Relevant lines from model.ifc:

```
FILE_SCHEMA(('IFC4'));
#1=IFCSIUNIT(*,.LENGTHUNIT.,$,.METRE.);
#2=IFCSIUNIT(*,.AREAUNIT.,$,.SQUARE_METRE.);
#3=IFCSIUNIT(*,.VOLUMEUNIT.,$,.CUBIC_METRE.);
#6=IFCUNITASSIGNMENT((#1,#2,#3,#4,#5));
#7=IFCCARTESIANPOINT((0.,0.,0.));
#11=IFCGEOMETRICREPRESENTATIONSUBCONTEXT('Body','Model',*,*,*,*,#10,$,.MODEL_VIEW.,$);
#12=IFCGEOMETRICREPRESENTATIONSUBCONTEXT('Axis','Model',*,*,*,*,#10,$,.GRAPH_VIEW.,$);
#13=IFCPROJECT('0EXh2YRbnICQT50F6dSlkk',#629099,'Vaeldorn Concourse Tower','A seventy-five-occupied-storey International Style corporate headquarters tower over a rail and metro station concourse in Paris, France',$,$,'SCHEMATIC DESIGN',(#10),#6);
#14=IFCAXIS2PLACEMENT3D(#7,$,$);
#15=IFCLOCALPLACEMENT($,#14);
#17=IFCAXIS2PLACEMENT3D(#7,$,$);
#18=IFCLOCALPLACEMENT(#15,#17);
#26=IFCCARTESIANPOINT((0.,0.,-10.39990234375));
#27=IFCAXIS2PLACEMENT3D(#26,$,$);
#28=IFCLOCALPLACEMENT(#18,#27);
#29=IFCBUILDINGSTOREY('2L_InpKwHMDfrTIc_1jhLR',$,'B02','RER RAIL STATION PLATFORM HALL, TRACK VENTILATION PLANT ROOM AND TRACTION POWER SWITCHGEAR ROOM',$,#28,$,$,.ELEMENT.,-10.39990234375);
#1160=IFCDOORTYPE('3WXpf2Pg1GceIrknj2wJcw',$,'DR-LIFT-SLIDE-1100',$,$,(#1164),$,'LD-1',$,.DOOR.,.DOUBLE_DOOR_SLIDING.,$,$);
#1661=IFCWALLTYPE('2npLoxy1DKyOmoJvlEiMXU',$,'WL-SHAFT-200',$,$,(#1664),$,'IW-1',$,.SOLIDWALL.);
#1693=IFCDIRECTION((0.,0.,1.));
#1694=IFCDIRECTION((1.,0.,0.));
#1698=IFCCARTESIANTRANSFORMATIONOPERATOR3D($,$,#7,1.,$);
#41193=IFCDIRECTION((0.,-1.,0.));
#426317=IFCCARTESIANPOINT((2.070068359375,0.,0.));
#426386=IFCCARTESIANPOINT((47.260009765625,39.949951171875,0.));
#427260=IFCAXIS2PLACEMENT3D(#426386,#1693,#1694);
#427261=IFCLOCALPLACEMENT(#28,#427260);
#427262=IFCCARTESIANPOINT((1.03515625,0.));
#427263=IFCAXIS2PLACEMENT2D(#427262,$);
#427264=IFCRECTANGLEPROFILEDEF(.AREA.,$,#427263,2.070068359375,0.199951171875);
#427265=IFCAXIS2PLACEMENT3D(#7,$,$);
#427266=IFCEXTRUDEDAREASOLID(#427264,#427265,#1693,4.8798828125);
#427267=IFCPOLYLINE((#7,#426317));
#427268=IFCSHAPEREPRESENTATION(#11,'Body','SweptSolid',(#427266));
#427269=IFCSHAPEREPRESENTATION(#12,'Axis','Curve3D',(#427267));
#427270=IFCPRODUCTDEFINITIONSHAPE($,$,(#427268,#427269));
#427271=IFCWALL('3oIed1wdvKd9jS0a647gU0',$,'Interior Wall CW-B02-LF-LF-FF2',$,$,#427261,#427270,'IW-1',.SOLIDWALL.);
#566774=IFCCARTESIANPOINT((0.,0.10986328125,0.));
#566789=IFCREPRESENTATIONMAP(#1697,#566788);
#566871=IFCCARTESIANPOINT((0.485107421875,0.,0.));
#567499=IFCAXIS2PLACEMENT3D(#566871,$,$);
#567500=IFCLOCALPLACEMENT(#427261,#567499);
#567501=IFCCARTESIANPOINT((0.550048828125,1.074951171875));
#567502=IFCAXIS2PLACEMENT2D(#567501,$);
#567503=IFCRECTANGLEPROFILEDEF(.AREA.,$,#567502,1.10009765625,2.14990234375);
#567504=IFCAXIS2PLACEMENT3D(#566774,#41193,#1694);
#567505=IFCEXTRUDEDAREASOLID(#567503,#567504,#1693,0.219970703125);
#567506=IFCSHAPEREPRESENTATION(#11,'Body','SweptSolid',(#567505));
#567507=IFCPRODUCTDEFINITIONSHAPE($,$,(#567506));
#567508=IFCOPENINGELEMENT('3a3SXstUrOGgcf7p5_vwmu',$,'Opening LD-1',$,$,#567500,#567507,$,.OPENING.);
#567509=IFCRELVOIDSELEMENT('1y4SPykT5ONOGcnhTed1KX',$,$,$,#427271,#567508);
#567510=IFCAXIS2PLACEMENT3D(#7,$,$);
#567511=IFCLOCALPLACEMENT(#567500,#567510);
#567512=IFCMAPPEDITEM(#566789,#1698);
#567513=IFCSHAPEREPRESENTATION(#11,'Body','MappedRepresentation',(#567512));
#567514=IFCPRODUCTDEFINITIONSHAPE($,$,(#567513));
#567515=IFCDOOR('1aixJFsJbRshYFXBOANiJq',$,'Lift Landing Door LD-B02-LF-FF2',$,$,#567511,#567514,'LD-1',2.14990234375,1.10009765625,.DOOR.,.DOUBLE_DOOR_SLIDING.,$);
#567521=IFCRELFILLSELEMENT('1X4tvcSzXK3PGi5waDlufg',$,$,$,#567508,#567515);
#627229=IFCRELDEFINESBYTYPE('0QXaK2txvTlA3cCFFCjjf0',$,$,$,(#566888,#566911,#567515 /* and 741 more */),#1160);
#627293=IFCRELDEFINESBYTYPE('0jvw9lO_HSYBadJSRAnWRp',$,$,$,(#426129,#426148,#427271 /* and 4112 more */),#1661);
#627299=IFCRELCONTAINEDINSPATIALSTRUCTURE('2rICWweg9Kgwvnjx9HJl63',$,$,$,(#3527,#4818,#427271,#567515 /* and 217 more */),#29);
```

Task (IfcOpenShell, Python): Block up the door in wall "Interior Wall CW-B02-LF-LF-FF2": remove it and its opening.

```python
import ifcopenshell
import ifcopenshell.api.feature
import ifcopenshell.api.root
import ifcopenshell.geom
import ifcopenshell.util.shape

model = ifcopenshell.open("model.ifc")
settings = ifcopenshell.geom.settings()


def volume(element):
    """Net volume in cubic metres, openings subtracted."""
    shape = ifcopenshell.geom.create_shape(settings, element)
    return ifcopenshell.util.shape.get_volume(shape.geometry)


door = model.by_guid("1aixJFsJbRshYFXBOANiJq")
opening = door.FillsVoids[0].RelatingOpeningElement
wall = opening.VoidsElements[0].RelatingBuildingElement
before = volume(wall)

ifcopenshell.api.root.remove_product(model, product=door)
ifcopenshell.api.feature.remove_feature(model, feature=opening)

after = volume(wall)

print(f"wall volume {before:.3f} -> {after:.3f} m3")

model.write("model_updated.ifc")
```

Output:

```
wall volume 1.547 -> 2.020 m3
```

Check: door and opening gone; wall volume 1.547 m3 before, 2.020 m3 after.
